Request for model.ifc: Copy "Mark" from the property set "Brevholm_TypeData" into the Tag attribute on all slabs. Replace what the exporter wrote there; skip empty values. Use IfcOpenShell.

First a look at what the model holds.

```python
import ifcopenshell
import ifcopenshell.util.element

model = ifcopenshell.open("model.ifc")
print(model.schema)
slabs = model.by_type("IfcSlab")
print(len(slabs), "slabs")
for e in slabs[:8]:
    source = ifcopenshell.util.element.get_pset(e, "Brevholm_TypeData", "Mark")
    target = e.Tag
    print(e.id(), repr(source), repr(target), sep=" | ")
```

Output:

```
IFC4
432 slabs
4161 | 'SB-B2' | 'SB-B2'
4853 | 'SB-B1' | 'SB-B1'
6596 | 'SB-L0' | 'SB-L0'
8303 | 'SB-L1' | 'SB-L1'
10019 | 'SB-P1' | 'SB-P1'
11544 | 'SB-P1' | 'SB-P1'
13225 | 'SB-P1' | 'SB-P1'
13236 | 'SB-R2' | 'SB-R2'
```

```python
import ifcopenshell
import ifcopenshell.util.element

model = ifcopenshell.open("model.ifc")

count = 0
for e in model.by_type("IfcSlab"):
    value = ifcopenshell.util.element.get_pset(e, "Brevholm_TypeData", "Mark")
    current = e.Tag
    if not value or not value.strip() or current == value:
        continue
    e.Tag = value
    count += 1

print(count, "slabs updated")

model.write("model_v2.ifc")
```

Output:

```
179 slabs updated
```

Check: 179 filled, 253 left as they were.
